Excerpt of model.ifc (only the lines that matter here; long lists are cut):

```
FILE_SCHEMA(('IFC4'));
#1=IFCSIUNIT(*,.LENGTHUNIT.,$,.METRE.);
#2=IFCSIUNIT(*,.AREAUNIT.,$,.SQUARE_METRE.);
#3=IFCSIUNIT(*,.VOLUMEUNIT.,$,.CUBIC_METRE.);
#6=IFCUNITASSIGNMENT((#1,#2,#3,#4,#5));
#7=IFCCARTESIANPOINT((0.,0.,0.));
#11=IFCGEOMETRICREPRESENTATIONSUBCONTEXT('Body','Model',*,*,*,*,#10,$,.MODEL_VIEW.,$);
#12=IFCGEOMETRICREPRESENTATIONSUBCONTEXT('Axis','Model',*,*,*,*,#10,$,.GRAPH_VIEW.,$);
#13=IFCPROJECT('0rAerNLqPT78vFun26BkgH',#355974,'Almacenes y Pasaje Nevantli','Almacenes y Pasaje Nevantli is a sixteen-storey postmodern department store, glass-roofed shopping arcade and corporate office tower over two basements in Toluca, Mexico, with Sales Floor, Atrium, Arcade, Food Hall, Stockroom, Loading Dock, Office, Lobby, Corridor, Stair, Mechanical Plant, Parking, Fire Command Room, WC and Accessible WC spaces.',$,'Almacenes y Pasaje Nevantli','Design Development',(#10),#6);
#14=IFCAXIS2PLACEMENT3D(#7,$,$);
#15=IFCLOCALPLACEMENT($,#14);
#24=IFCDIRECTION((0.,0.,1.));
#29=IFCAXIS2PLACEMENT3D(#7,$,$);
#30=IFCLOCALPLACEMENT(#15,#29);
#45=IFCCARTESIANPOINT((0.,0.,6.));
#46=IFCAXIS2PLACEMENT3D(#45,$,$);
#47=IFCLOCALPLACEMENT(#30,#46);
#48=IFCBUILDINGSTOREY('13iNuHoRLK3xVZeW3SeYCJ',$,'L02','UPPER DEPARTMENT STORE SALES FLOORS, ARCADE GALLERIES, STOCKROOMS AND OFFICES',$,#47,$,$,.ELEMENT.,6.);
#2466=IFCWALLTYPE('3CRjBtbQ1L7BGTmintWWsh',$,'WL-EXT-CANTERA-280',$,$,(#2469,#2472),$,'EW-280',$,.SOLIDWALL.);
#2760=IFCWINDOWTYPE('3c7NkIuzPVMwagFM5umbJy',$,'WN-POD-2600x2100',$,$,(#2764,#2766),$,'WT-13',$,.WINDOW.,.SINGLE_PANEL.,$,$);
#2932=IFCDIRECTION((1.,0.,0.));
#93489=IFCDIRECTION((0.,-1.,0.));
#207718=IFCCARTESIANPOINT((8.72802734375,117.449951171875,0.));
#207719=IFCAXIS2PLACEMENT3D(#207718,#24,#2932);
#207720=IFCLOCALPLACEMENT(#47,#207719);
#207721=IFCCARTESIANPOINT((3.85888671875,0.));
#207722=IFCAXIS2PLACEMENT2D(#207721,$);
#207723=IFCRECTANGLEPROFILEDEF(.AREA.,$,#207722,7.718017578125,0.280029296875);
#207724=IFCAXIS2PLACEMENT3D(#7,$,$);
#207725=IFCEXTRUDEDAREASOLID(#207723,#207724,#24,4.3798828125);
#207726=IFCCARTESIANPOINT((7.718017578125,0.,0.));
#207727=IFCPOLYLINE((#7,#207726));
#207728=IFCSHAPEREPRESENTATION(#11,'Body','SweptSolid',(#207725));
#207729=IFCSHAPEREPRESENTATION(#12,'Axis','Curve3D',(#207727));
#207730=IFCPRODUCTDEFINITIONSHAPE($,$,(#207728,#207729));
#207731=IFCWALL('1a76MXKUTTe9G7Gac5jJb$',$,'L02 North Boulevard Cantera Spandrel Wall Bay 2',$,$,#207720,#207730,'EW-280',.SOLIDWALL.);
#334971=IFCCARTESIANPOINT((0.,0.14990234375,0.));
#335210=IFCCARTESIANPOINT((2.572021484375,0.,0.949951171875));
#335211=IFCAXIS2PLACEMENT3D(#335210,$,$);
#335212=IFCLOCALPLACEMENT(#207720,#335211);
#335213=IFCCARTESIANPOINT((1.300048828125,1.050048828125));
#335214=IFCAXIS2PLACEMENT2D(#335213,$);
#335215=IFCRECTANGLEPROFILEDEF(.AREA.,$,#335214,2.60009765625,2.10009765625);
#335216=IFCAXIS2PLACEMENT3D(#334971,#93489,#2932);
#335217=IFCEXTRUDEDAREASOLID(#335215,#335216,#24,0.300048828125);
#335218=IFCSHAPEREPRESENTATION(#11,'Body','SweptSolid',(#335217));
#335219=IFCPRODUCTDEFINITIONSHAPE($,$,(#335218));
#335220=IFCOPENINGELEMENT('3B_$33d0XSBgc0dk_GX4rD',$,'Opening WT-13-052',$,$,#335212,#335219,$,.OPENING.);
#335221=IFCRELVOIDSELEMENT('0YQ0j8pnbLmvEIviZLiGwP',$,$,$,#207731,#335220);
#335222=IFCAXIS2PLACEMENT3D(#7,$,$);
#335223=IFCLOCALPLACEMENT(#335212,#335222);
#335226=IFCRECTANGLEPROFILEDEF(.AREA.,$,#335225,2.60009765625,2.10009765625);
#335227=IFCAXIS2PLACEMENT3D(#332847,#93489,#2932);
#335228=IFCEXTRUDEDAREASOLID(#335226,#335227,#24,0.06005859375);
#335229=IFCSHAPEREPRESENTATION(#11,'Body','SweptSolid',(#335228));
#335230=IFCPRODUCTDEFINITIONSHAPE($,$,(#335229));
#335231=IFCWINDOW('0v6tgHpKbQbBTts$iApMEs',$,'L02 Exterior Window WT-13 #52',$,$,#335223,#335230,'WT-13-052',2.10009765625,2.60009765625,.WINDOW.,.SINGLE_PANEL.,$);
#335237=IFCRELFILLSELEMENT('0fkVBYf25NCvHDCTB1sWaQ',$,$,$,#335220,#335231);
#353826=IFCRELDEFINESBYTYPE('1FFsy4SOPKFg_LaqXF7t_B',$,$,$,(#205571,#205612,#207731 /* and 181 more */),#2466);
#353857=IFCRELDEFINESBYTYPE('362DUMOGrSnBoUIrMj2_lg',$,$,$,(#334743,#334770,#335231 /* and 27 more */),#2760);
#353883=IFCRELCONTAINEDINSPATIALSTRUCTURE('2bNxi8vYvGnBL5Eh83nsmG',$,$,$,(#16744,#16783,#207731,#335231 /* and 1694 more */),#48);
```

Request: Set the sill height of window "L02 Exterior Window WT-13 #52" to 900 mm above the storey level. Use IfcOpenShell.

```python
import numpy as np
import ifcopenshell
import ifcopenshell.api.geometry
import ifcopenshell.geom
import ifcopenshell.util.element
import ifcopenshell.util.placement
import ifcopenshell.util.shape
import ifcopenshell.util.unit

model = ifcopenshell.open("model.ifc")
unit_scale = ifcopenshell.util.unit.calculate_unit_scale(model)

window = model.by_guid("0v6tgHpKbQbBTts$iApMEs")
opening = window.FillsVoids[0].RelatingOpeningElement
storey = ifcopenshell.util.element.get_container(window, ifc_class="IfcBuildingStorey")
level = ifcopenshell.util.placement.get_local_placement(storey.ObjectPlacement)[2, 3]

# The opening's origin need not be at the sill, so measure its lowest point.
shape = ifcopenshell.geom.create_shape(ifcopenshell.geom.settings(), opening)
bottom = ifcopenshell.util.shape.get_shape_bottom_elevation(shape, shape.geometry) / unit_scale
dz = level + 0.9 / unit_scale - bottom

shift = np.array([0.0, 0.0, dz])
# The window is placed relative to its opening, so it follows when the opening moves.
matrix = ifcopenshell.util.placement.get_local_placement(opening.ObjectPlacement)
matrix[:3, 3] += shift
ifcopenshell.api.geometry.edit_object_placement(
    model, product=opening, matrix=matrix, is_si=False, should_transform_children=True
)

print(f"moved by {dz * unit_scale:+.3f} m")

model.write("model_edited.ifc")
```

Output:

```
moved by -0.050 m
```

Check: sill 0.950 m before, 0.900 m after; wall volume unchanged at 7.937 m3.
